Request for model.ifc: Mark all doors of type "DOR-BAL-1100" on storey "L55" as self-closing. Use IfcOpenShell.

First a look at what the model holds.

```python
import ifcopenshell
import ifcopenshell.util.element

model = ifcopenshell.open("model.ifc")
print(model.schema)
storey = next(s for s in model.by_type("IfcBuildingStorey") if s.Name == "L55")
doors = [e for e in ifcopenshell.util.element.get_decomposition(storey) if e.is_a("IfcDoor")]
seen = {}
for e in doors:
    element_type = ifcopenshell.util.element.get_type(e)
    key = (element_type.Name if element_type != e and element_type else None, ifcopenshell.util.element.get_pset(e, "Pset_DoorCommon", "SelfClosing"))
    seen[key] = seen.get(key, 0) + 1
for (name, value), count in sorted(seen.items(), key=str):
    print(count, "x", name, "|", value)
```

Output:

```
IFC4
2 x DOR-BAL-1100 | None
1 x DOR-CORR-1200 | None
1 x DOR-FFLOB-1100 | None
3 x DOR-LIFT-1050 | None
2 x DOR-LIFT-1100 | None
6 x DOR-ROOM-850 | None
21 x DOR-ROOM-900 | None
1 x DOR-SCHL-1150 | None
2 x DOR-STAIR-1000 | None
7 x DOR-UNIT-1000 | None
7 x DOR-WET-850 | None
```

```python
import ifcopenshell
import ifcopenshell.api.pset
import ifcopenshell.util.element

model = ifcopenshell.open("model.ifc")

storey = next(s for s in model.by_type("IfcBuildingStorey") if s.Name == "L55")
doors = [e for e in ifcopenshell.util.element.get_decomposition(storey) if e.is_a("IfcDoor")]

count = 0
for e in doors:
    element_type = ifcopenshell.util.element.get_type(e)
    if element_type in (None, e) or element_type.Name != "DOR-BAL-1100":
        continue
    # add_pset returns the element's existing set when there is one.
    pset = ifcopenshell.api.pset.add_pset(model, product=e, name="Pset_DoorCommon")
    ifcopenshell.api.pset.edit_pset(model, pset=pset, properties={"SelfClosing": True})
    count += 1

print(count, "doors updated")

model.write("model_updated.ifc")
```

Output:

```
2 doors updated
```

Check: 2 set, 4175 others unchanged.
